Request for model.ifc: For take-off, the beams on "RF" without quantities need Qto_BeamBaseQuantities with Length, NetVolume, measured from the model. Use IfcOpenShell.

First a look at what the model holds.

```python
import ifcopenshell
import ifcopenshell.util.element
import ifcopenshell.util.unit

model = ifcopenshell.open("model.ifc")
print(model.schema)
for unit_type in ("LENGTHUNIT", "AREAUNIT", "VOLUMEUNIT"):
    print(unit_type, ifcopenshell.util.unit.calculate_unit_scale(model, unit_type))
storey = next(s for s in model.by_type("IfcBuildingStorey") if s.Name == "RF")
beams = [e for e in ifcopenshell.util.element.get_decomposition(storey) if e.is_a("IfcBeam")]
for e in sorted(beams, key=lambda e: e.id()):
    print(e.id(), e.is_a(), e.Name, list(ifcopenshell.util.element.get_psets(e, qtos_only=True)), sep=" | ")
```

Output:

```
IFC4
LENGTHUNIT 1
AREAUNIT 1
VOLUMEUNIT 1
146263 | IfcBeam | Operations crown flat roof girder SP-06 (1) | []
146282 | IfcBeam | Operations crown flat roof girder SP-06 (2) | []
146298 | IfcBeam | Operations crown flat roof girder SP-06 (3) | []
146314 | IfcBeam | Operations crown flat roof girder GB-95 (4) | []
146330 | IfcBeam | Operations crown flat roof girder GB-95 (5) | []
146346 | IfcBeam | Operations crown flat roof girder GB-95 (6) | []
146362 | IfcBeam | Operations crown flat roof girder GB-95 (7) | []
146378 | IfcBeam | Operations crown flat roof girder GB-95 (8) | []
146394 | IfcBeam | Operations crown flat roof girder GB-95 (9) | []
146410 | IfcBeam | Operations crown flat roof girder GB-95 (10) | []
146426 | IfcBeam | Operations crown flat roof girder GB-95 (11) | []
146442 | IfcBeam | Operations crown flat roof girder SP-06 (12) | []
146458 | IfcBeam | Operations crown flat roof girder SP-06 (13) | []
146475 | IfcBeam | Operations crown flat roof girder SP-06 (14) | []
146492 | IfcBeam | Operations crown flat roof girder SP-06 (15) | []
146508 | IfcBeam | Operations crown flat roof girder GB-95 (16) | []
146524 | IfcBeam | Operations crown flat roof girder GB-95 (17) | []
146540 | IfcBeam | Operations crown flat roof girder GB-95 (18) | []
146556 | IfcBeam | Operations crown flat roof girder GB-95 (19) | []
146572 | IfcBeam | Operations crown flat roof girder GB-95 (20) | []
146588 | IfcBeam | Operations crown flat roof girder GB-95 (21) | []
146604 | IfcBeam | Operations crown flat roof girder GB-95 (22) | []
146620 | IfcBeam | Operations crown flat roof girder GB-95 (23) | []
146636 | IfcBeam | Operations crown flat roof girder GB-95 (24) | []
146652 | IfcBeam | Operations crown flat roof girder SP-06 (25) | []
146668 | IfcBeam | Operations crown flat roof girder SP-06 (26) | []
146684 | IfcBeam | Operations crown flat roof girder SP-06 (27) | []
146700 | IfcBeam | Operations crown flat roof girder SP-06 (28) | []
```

```python
import ifcopenshell
import ifcopenshell.api.pset
import ifcopenshell.geom
import ifcopenshell.util.element
import ifcopenshell.util.shape
import ifcopenshell.util.unit

model = ifcopenshell.open("model.ifc")
unit_scale = ifcopenshell.util.unit.calculate_unit_scale(model)
volume_scale = ifcopenshell.util.unit.calculate_unit_scale(model, "VOLUMEUNIT")
settings = ifcopenshell.geom.settings()

storey = next(s for s in model.by_type("IfcBuildingStorey") if s.Name == "RF")
beams = [e for e in ifcopenshell.util.element.get_decomposition(storey) if e.is_a("IfcBeam")]

for e in sorted(beams, key=lambda e: e.id()):
    if ifcopenshell.util.element.get_psets(e, qtos_only=True, should_inherit=False):
        continue
    # Geometry comes back in metres, in the element's own axes.
    shape = ifcopenshell.geom.create_shape(settings, e)
    values = {
        "Length": ifcopenshell.util.shape.get_max_xyz(shape.geometry) / unit_scale,
        "NetVolume": ifcopenshell.util.shape.get_volume(shape.geometry) / volume_scale,
    }
    qto = ifcopenshell.api.pset.add_qto(model, product=e, name="Qto_BeamBaseQuantities")
    ifcopenshell.api.pset.edit_qto(model, qto=qto, properties=values)
    print(e.id(), {k: round(v, 3) for k, v in values.items()})

model.write("model-out.ifc")
```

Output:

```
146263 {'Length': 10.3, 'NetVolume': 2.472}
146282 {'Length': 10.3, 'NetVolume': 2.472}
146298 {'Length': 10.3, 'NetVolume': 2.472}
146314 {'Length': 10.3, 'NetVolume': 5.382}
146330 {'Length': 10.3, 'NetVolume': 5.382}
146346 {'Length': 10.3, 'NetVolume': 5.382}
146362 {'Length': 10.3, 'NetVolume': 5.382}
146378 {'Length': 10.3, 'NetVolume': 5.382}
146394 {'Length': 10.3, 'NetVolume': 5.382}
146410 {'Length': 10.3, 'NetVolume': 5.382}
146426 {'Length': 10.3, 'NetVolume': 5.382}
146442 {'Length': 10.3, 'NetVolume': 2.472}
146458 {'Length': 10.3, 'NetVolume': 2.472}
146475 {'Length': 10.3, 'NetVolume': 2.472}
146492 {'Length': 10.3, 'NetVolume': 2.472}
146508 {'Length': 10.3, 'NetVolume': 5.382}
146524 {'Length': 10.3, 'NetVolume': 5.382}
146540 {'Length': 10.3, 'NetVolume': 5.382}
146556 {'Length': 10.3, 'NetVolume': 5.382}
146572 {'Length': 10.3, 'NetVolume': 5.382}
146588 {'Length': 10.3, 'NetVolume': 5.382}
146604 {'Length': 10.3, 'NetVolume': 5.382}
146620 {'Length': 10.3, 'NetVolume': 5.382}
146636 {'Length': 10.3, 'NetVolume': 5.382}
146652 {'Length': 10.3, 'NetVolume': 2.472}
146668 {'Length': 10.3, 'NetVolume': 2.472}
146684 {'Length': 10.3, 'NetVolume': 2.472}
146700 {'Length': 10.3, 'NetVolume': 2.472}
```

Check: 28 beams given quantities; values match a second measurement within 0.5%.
